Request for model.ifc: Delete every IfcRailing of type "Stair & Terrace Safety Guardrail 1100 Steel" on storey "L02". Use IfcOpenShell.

First a look at what the model holds.

```python
import ifcopenshell
import ifcopenshell.util.element

model = ifcopenshell.open("model.ifc")
print(model.schema)
storey = next(s for s in model.by_type("IfcBuildingStorey") if s.Name == "L02")
railings = [e for e in ifcopenshell.util.element.get_decomposition(storey) if e.is_a("IfcRailing")]
seen = {}
for e in railings:
    element_type = ifcopenshell.util.element.get_type(e)
    name = element_type.Name if element_type not in (None, e) else None
    seen[name] = seen.get(name, 0) + 1
for name, count in sorted(seen.items(), key=str):
    print(count, "x", name)
```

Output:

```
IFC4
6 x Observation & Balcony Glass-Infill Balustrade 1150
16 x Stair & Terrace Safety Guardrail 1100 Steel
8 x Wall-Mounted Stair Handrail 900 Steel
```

```python
import ifcopenshell
import ifcopenshell.api.root
import ifcopenshell.util.element

model = ifcopenshell.open("model.ifc")

storey = next(s for s in model.by_type("IfcBuildingStorey") if s.Name == "L02")
railings = [e for e in ifcopenshell.util.element.get_decomposition(storey) if e.is_a("IfcRailing")]
targets = [e for e in railings if (t := ifcopenshell.util.element.get_type(e)) not in (None, e) and t.Name == "Stair & Terrace Safety Guardrail 1100 Steel"]

for e in targets:
    ifcopenshell.api.root.remove_product(model, product=e)
print(len(targets), "removed")

model.write("model_updated.ifc")
```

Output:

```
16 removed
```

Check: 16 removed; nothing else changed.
